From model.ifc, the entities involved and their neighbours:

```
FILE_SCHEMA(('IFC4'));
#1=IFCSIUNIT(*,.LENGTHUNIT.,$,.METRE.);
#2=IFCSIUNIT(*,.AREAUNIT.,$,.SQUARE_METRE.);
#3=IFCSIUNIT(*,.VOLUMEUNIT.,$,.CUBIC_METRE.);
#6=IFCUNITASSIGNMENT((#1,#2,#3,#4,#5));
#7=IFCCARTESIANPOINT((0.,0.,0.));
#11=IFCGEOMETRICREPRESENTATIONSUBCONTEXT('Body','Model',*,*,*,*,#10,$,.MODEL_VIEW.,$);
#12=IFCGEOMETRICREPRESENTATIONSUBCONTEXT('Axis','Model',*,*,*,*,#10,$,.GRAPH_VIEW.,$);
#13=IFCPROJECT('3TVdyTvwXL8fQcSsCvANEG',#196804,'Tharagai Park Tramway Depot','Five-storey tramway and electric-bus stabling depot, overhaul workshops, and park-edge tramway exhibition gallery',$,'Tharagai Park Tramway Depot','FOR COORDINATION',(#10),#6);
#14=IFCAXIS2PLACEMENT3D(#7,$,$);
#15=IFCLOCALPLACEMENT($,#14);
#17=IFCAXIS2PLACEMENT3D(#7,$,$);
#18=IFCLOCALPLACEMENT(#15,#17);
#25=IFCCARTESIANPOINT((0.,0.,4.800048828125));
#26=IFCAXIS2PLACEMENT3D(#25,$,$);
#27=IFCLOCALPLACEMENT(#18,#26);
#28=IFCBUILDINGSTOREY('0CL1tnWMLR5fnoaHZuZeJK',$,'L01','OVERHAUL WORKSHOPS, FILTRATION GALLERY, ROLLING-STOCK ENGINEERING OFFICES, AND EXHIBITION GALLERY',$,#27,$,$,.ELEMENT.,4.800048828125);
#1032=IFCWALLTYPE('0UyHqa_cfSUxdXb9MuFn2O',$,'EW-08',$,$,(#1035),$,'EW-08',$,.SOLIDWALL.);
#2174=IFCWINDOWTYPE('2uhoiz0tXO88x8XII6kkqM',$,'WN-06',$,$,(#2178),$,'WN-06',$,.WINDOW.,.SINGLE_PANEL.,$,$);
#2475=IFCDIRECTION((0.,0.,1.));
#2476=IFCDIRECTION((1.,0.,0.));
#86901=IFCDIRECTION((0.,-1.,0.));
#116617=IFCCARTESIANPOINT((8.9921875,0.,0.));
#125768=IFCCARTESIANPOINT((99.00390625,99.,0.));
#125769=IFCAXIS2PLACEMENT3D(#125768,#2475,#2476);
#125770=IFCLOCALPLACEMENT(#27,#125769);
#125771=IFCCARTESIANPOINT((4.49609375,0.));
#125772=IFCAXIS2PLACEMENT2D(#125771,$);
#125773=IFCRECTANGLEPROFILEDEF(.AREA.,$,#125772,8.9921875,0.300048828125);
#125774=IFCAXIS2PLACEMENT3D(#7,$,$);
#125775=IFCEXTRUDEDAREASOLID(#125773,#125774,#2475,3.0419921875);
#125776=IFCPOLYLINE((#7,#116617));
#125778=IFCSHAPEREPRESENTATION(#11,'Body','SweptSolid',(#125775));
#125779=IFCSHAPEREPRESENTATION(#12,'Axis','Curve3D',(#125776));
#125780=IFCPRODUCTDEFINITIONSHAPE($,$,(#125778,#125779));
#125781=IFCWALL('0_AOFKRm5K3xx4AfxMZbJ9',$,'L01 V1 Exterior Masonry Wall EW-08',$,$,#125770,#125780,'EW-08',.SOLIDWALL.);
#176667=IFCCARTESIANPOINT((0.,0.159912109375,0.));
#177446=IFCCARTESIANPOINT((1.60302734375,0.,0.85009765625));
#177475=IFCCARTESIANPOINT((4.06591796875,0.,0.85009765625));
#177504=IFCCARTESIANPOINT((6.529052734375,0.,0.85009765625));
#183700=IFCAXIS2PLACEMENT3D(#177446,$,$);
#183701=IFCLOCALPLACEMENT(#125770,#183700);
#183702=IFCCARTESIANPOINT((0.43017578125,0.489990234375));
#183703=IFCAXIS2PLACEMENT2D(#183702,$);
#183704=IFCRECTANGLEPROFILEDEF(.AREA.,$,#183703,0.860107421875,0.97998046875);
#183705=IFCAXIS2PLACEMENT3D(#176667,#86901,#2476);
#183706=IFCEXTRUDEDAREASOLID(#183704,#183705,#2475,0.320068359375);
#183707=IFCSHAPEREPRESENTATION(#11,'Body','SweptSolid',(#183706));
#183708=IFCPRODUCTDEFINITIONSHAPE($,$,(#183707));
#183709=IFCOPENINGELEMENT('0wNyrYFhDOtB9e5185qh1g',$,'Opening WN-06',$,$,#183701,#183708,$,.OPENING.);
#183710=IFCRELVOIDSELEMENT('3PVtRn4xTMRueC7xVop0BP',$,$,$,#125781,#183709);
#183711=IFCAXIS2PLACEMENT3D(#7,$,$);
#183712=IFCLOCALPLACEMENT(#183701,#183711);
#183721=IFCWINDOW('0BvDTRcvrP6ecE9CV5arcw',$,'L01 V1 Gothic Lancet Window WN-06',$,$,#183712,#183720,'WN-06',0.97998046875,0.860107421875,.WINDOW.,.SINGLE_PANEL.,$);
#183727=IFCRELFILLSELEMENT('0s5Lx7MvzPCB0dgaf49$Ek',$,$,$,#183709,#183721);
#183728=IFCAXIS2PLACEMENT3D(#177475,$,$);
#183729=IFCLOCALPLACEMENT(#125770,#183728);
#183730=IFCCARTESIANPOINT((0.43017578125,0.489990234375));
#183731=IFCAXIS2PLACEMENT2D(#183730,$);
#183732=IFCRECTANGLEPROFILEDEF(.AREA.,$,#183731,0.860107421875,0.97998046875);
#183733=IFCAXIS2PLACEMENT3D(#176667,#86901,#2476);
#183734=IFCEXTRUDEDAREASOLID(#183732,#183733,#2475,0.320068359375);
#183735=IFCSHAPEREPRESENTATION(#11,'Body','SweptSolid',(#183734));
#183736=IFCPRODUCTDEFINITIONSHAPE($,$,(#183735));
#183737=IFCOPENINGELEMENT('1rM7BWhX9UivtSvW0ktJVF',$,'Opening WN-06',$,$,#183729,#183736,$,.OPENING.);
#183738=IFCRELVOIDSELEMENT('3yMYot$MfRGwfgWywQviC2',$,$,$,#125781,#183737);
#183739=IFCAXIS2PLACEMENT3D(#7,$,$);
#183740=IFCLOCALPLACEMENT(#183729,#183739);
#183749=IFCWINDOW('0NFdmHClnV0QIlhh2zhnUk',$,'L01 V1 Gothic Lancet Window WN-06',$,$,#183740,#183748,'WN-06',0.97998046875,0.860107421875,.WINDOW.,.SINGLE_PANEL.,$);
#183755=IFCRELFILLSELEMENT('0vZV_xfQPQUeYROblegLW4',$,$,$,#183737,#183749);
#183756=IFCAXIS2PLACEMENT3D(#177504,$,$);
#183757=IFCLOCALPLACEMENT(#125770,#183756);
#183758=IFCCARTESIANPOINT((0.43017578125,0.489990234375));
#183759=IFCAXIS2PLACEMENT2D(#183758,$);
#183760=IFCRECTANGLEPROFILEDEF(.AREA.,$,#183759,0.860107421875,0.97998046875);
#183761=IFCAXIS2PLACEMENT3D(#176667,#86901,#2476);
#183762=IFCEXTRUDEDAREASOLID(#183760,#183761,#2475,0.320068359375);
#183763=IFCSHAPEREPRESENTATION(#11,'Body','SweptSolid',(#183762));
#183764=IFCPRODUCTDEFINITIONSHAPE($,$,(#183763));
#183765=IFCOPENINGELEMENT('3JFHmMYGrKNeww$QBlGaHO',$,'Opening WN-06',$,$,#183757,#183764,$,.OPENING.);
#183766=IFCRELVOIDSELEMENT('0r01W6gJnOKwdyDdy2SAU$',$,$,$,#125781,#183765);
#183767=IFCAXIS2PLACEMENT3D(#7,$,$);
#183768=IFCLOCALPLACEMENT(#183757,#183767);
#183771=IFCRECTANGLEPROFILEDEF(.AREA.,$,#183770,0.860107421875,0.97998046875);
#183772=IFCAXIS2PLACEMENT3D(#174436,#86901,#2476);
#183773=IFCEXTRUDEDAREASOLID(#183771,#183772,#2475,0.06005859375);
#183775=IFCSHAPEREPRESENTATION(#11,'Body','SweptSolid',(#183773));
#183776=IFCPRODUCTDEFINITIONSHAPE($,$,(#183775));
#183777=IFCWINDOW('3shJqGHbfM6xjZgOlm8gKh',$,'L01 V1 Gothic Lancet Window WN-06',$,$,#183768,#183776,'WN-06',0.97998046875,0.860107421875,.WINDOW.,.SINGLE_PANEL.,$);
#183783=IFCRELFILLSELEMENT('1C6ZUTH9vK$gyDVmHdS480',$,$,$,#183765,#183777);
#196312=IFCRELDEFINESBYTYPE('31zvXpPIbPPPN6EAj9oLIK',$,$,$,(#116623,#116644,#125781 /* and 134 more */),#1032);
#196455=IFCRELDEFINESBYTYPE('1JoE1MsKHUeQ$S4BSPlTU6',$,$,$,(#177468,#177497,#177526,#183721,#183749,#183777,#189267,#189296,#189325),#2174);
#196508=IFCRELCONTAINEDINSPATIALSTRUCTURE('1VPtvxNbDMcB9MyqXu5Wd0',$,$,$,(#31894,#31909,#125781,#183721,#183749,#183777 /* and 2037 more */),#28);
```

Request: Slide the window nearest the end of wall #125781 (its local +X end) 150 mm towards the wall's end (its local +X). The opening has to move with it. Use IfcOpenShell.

```python
import ifcopenshell
import ifcopenshell.api.geometry
import ifcopenshell.util.placement
import ifcopenshell.util.unit

model = ifcopenshell.open("model.ifc")
unit_scale = ifcopenshell.util.unit.calculate_unit_scale(model)

window = model.by_guid("3shJqGHbfM6xjZgOlm8gKh")
opening = window.FillsVoids[0].RelatingOpeningElement
wall = opening.VoidsElements[0].RelatingBuildingElement

wall_matrix = ifcopenshell.util.placement.get_local_placement(wall.ObjectPlacement)
shift = wall_matrix[:3, 0] * 0.15 / unit_scale
before = ifcopenshell.util.placement.get_local_placement(window.ObjectPlacement)[:3, 3].copy()

# The window is placed relative to its opening, so it follows when the opening moves.
matrix = ifcopenshell.util.placement.get_local_placement(opening.ObjectPlacement)
matrix[:3, 3] += shift
ifcopenshell.api.geometry.edit_object_placement(
    model, product=opening, matrix=matrix, is_si=False, should_transform_children=True
)

after = ifcopenshell.util.placement.get_local_placement(window.ObjectPlacement)[:3, 3]
print("window moved by", (after - before).round(3) + 0.0)

model.write("model_v2.ifc")
```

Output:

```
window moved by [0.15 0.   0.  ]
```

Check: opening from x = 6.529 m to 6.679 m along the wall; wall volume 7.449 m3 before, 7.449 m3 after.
